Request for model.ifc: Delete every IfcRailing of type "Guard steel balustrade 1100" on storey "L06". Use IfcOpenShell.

First a look at what the model holds.

```python
import ifcopenshell
import ifcopenshell.util.element

model = ifcopenshell.open("model.ifc")
print(model.schema)
storey = next(s for s in model.by_type("IfcBuildingStorey") if s.Name == "L06")
railings = [e for e in ifcopenshell.util.element.get_decomposition(storey) if e.is_a("IfcRailing")]
seen = {}
for e in railings:
    element_type = ifcopenshell.util.element.get_type(e)
    name = element_type.Name if element_type not in (None, e) else None
    seen[name] = seen.get(name, 0) + 1
for name, count in sorted(seen.items(), key=str):
    print(count, "x", name)
```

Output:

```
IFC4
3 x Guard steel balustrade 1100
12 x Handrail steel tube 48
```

```python
import ifcopenshell
import ifcopenshell.api.root
import ifcopenshell.util.element

model = ifcopenshell.open("model.ifc")

storey = next(s for s in model.by_type("IfcBuildingStorey") if s.Name == "L06")
railings = [e for e in ifcopenshell.util.element.get_decomposition(storey) if e.is_a("IfcRailing")]
targets = [e for e in railings if (t := ifcopenshell.util.element.get_type(e)) not in (None, e) and t.Name == "Guard steel balustrade 1100"]

for e in targets:
    ifcopenshell.api.root.remove_product(model, product=e)
print(len(targets), "removed")

model.write("model_edited.ifc")
```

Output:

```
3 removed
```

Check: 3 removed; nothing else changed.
